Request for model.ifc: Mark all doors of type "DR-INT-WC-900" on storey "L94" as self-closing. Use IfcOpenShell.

First a look at what the model holds.

```python
import ifcopenshell
import ifcopenshell.util.element

model = ifcopenshell.open("model.ifc")
print(model.schema)
storey = next(s for s in model.by_type("IfcBuildingStorey") if s.Name == "L94")
doors = [e for e in ifcopenshell.util.element.get_decomposition(storey) if e.is_a("IfcDoor")]
seen = {}
for e in doors:
    element_type = ifcopenshell.util.element.get_type(e)
    key = (element_type.Name if element_type != e and element_type else None, ifcopenshell.util.element.get_pset(e, "Pset_DoorCommon", "SelfClosing"))
    seen[key] = seen.get(key, 0) + 1
for (name, value), count in sorted(seen.items(), key=str):
    print(count, "x", name, "|", value)
```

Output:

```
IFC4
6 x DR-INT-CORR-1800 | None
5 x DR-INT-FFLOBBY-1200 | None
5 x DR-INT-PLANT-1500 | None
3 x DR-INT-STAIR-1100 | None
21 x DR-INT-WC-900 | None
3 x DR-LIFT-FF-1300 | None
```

```python
import ifcopenshell
import ifcopenshell.api.pset
import ifcopenshell.util.element

model = ifcopenshell.open("model.ifc")

storey = next(s for s in model.by_type("IfcBuildingStorey") if s.Name == "L94")
doors = [e for e in ifcopenshell.util.element.get_decomposition(storey) if e.is_a("IfcDoor")]

count = 0
for e in doors:
    element_type = ifcopenshell.util.element.get_type(e)
    if element_type in (None, e) or element_type.Name != "DR-INT-WC-900":
        continue
    found = ifcopenshell.util.element.get_pset(e, "Pset_DoorCommon", should_inherit=False)
    if found:
        pset = model.by_id(found["id"])
        if len(ifcopenshell.util.element.get_elements_by_pset(pset)) > 1:
            pset = ifcopenshell.api.pset.unshare_pset(model, products=[e], pset=pset)[0]
    else:
        pset = ifcopenshell.api.pset.add_pset(model, product=e, name="Pset_DoorCommon")
    ifcopenshell.api.pset.edit_pset(model, pset=pset, properties={"SelfClosing": True})
    count += 1

print(count, "doors updated")

model.write("model_rev.ifc")
```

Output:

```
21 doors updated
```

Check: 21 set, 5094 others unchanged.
